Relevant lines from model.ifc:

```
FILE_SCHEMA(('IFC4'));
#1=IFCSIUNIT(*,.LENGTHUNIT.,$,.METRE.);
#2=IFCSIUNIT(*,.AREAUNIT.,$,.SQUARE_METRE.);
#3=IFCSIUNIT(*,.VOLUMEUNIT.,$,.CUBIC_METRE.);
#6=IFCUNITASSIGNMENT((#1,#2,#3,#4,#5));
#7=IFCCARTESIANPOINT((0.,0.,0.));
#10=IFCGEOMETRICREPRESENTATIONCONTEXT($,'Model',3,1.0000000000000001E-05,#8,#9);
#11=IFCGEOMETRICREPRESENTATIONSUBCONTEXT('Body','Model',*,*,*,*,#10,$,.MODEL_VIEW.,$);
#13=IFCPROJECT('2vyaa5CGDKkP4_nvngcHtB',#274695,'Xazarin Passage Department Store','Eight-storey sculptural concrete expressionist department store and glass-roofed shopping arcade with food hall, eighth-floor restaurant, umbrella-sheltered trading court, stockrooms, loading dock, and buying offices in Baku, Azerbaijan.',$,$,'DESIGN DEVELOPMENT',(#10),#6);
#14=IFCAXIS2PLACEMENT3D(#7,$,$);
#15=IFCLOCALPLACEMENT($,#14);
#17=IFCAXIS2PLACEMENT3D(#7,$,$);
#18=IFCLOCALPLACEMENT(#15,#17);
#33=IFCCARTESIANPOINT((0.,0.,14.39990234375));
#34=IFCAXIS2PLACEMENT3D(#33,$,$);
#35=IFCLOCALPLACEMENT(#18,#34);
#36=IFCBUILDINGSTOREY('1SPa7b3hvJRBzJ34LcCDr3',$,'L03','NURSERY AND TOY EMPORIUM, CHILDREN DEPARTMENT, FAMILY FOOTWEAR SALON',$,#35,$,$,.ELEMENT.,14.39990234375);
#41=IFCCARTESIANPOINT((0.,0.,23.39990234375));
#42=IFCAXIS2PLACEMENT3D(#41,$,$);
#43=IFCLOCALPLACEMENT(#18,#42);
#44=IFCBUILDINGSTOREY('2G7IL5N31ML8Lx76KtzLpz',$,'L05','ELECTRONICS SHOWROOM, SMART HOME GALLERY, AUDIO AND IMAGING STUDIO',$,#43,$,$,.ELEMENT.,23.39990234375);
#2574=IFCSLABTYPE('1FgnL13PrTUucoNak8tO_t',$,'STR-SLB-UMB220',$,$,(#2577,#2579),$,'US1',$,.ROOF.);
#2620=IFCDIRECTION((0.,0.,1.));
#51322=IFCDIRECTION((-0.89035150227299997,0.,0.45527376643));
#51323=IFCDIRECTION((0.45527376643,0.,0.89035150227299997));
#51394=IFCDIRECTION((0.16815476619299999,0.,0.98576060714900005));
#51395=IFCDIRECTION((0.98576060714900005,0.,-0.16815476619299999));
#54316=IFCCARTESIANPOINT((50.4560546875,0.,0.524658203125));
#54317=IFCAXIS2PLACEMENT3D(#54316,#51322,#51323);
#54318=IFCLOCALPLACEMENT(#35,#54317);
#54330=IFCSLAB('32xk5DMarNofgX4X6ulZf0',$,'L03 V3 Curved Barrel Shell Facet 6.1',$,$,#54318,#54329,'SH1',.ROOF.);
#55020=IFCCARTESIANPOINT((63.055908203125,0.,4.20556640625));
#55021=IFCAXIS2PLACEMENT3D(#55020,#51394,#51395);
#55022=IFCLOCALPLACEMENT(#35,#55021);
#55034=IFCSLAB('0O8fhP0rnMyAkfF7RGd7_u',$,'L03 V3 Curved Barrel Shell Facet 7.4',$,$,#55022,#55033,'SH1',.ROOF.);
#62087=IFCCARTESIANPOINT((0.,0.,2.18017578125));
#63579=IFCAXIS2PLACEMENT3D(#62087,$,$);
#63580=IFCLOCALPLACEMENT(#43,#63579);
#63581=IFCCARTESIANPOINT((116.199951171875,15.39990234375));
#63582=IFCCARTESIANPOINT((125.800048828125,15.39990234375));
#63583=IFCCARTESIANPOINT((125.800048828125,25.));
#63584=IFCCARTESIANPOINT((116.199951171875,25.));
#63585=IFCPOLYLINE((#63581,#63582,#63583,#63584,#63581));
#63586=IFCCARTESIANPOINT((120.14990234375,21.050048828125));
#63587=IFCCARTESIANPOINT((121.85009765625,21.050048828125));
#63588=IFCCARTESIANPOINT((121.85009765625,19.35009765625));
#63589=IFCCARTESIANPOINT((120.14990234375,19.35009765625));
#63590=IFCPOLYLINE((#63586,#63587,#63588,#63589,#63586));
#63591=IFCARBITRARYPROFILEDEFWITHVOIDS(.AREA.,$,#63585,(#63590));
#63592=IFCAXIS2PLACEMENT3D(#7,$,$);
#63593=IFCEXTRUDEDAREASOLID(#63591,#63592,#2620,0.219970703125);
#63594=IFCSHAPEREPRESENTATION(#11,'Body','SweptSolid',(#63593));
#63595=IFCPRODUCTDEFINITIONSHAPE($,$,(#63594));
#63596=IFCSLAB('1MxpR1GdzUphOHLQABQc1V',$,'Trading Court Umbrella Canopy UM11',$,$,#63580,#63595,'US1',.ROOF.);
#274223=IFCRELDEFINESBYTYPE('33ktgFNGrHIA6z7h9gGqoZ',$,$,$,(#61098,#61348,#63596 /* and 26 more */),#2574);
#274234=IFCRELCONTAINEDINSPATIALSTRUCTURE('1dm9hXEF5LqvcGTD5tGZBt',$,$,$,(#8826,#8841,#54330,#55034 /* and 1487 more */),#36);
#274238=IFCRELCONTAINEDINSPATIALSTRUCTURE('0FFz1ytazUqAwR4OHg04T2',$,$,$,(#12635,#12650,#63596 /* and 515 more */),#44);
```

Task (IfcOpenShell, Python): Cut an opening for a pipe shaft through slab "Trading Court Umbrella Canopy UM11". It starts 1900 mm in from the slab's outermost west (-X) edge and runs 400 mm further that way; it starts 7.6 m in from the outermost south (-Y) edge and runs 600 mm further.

```python
import numpy as np
import ifcopenshell
import ifcopenshell.api.feature
import ifcopenshell.api.geometry
import ifcopenshell.api.root
import ifcopenshell.geom
import ifcopenshell.util.placement
import ifcopenshell.util.representation
import ifcopenshell.util.shape
import ifcopenshell.util.unit

model = ifcopenshell.open("model.ifc")
unit_scale = ifcopenshell.util.unit.calculate_unit_scale(model)
settings = ifcopenshell.geom.settings()


def volume(element):
    """Net volume in cubic metres, openings subtracted."""
    shape = ifcopenshell.geom.create_shape(settings, element)
    return ifcopenshell.util.shape.get_volume(shape.geometry)


slab = model.by_guid("1MxpR1GdzUphOHLQABQc1V")
before = volume(slab)

# Extent in the slab's own axes, in metres. The edges named are its -X and -Y sides.
slab_shape = ifcopenshell.geom.create_shape(settings, slab)
vertices = ifcopenshell.util.shape.get_vertices(slab_shape.geometry)
x_min, y_min, bottom = vertices.min(axis=0)
top = vertices[:, 2].max()

opening = ifcopenshell.api.root.create_entity(model, ifc_class="IfcOpeningElement", name="Pipe shaft opening", predefined_type="OPENING")
context = ifcopenshell.util.representation.get_context(model, "Model", "Body", "MODEL_VIEW")
width, depth = 0.4, 0.6
outline = [(0.0, 0.0), (width, 0.0), (width, depth), (0.0, depth), (0.0, 0.0)]
# Overshoot both faces by 50 mm so the cut is clean.
shape = ifcopenshell.api.geometry.add_slab_representation(
    model, context=context, depth=top - bottom + 0.1, polyline=outline
)
ifcopenshell.api.geometry.assign_representation(model, product=opening, representation=shape)

matrix = ifcopenshell.util.placement.get_local_placement(slab.ObjectPlacement)
matrix[:, 3] = matrix @ np.append(np.array([x_min + 1.9, y_min + 7.6, bottom - 0.05]) / unit_scale, 1.0)
ifcopenshell.api.geometry.edit_object_placement(model, product=opening, matrix=matrix, is_si=False)
ifcopenshell.api.feature.add_feature(model, feature=opening, element=slab)

after = volume(slab)

print(f"slab volume {before:.3f} -> {after:.3f} m3")

model.write("model_v2.ifc")
```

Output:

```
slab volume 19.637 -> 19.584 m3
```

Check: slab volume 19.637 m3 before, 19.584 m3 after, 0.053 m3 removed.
